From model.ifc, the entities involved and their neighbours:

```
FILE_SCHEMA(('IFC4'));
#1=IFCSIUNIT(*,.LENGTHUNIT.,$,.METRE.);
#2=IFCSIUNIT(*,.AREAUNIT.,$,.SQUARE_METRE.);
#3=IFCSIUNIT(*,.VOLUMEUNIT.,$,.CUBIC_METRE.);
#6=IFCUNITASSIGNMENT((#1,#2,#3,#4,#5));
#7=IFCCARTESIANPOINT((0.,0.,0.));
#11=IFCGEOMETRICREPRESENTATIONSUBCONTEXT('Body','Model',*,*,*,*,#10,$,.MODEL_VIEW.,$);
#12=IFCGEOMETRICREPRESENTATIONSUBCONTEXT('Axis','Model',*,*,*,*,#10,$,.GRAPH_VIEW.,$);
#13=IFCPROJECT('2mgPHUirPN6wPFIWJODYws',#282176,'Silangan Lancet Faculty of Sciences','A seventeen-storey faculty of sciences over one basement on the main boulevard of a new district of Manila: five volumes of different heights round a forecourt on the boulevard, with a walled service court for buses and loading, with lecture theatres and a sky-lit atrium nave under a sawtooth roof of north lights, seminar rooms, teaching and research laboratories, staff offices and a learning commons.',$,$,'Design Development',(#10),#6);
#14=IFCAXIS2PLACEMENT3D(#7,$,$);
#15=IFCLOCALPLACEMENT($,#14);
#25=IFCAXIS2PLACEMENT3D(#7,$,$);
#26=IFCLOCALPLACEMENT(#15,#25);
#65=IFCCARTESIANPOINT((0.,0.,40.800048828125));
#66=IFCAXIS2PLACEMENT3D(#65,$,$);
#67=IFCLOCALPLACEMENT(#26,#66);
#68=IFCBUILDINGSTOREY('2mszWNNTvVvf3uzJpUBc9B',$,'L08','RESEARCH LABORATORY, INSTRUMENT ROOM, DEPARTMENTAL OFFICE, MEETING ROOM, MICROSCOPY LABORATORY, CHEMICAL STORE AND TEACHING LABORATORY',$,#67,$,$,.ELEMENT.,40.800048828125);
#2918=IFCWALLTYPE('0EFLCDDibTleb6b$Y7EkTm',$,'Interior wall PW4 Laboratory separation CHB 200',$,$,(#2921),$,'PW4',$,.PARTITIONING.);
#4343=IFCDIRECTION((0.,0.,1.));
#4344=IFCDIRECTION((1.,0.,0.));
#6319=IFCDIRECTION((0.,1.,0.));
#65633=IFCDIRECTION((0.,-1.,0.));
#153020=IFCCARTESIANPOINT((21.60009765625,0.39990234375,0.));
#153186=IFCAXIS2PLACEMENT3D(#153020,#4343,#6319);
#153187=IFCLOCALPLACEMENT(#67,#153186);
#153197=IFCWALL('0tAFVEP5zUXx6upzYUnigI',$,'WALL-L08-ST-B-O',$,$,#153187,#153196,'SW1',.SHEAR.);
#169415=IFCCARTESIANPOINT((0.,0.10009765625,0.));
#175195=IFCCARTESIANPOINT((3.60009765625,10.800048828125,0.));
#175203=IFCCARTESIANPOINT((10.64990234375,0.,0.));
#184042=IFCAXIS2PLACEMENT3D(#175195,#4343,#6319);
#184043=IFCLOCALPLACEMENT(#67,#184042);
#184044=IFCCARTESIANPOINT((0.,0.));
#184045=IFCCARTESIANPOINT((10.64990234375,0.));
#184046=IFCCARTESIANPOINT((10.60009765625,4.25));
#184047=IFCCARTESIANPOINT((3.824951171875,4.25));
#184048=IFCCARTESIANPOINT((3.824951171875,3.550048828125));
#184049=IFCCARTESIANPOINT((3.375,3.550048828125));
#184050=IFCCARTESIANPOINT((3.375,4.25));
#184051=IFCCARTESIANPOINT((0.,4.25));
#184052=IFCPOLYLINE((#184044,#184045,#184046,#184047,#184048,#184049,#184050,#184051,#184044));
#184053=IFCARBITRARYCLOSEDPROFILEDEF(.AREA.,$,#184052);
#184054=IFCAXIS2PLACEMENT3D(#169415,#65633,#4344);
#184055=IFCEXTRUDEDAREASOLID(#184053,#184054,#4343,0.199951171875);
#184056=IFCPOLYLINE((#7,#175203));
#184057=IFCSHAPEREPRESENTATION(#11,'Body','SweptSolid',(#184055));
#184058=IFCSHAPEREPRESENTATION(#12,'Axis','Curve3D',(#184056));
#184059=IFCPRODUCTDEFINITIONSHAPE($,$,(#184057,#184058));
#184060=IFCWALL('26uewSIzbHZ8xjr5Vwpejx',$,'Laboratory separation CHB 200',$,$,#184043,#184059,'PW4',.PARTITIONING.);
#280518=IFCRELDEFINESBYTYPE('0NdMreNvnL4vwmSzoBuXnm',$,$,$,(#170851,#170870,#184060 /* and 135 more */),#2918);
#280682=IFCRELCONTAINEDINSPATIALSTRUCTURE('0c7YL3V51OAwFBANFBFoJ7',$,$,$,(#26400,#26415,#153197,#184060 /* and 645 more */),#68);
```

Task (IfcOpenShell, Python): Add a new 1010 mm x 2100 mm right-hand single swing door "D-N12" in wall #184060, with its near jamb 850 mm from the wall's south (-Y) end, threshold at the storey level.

```python
import numpy as np
import ifcopenshell
import ifcopenshell.api.feature
import ifcopenshell.api.geometry
import ifcopenshell.api.root
import ifcopenshell.api.spatial
import ifcopenshell.geom
import ifcopenshell.util.element
import ifcopenshell.util.placement
import ifcopenshell.util.representation
import ifcopenshell.util.shape
import ifcopenshell.util.unit

model = ifcopenshell.open("model.ifc")
unit_scale = ifcopenshell.util.unit.calculate_unit_scale(model)
settings = ifcopenshell.geom.settings()


def volume(element):
    """Net volume in cubic metres, openings subtracted."""
    shape = ifcopenshell.geom.create_shape(settings, element)
    return ifcopenshell.util.shape.get_volume(shape.geometry)


wall = model.by_guid("26uewSIzbHZ8xjr5Vwpejx")
storey = ifcopenshell.util.element.get_container(wall, ifc_class="IfcBuildingStorey")
context = ifcopenshell.util.representation.get_context(model, "Model", "Body", "MODEL_VIEW")
before = volume(wall)

width, height, from_end, sill = 1.01, 2.1, 0.85, 0.0  # metres

# The wall runs along its own X axis, and the end named is its -X end.
wall_shape = ifcopenshell.geom.create_shape(settings, wall)
x, y, z = ifcopenshell.util.shape.get_vertices(wall_shape.geometry).T
start = x.min() + from_end
face, thickness = float(y.min()), float(y.max() - y.min())
wall_matrix = ifcopenshell.util.placement.get_local_placement(wall.ObjectPlacement)
level = ifcopenshell.util.placement.get_local_placement(storey.ObjectPlacement)[2, 3]


def in_wall(x, y):
    """Placement at x, y metres in the wall's axes, at sill height."""
    matrix = wall_matrix.copy()
    matrix[:, 3] = wall_matrix @ np.array([x / unit_scale, y / unit_scale, 0.0, 1.0])
    matrix[2, 3] = level + sill / unit_scale
    return matrix


# Opening: a box that overshoots both wall faces by 50 mm.
opening = ifcopenshell.api.root.create_entity(model, ifc_class="IfcOpeningElement", predefined_type="OPENING")
box = ifcopenshell.api.geometry.add_wall_representation(
    model, context=context, length=width, height=height, thickness=thickness + 0.1
)
ifcopenshell.api.geometry.assign_representation(model, product=opening, representation=box)
ifcopenshell.api.geometry.edit_object_placement(model, product=opening, matrix=in_wall(start, face - 0.05), is_si=False)
ifcopenshell.api.feature.add_feature(model, feature=opening, element=wall)

door = ifcopenshell.api.root.create_entity(model, ifc_class="IfcDoor", name="D-N12", predefined_type="DOOR")
door.OverallWidth, door.OverallHeight = width / unit_scale, height / unit_scale
door.OperationType = "SINGLE_SWING_RIGHT"
body = ifcopenshell.api.geometry.add_door_representation(
    model,
    context=context,
    overall_width=door.OverallWidth,
    overall_height=door.OverallHeight,
    operation_type="SINGLE_SWING_RIGHT",
    lining_properties={"LiningDepth": thickness / unit_scale, "ThresholdDepth": thickness / unit_scale},
)
ifcopenshell.api.geometry.assign_representation(model, product=door, representation=body)
ifcopenshell.api.spatial.assign_container(model, products=[door], relating_structure=storey)
ifcopenshell.api.feature.add_filling(model, opening=opening, element=door)

# The lining spans the wall, so the door starts at the wall face.
ifcopenshell.api.geometry.edit_object_placement(model, product=door, matrix=in_wall(start, face), is_si=False)

after = volume(wall)

print(f"wall volume {before:.3f} -> {after:.3f} m3")

model.write("model_edited.ifc")
```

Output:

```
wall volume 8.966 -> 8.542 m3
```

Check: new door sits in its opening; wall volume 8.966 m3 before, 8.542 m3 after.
